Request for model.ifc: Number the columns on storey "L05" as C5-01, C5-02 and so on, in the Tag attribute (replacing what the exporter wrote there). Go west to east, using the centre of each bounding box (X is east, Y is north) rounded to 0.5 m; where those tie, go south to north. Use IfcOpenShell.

First a look at what the model holds.

```python
import ifcopenshell
import ifcopenshell.util.element
import ifcopenshell.util.placement

model = ifcopenshell.open("model.ifc")
print(model.schema)
storey = next(s for s in model.by_type("IfcBuildingStorey") if s.Name == "L05")
columns = [e for e in ifcopenshell.util.element.get_decomposition(storey) if e.is_a("IfcColumn")]
for e in sorted(columns, key=lambda e: e.id()):
    origin = ifcopenshell.util.placement.get_local_placement(e.ObjectPlacement)[:3, 3]
    print(e.id(), e.Tag, e.Name, origin.round(2) + 0.0, sep=" | ")
```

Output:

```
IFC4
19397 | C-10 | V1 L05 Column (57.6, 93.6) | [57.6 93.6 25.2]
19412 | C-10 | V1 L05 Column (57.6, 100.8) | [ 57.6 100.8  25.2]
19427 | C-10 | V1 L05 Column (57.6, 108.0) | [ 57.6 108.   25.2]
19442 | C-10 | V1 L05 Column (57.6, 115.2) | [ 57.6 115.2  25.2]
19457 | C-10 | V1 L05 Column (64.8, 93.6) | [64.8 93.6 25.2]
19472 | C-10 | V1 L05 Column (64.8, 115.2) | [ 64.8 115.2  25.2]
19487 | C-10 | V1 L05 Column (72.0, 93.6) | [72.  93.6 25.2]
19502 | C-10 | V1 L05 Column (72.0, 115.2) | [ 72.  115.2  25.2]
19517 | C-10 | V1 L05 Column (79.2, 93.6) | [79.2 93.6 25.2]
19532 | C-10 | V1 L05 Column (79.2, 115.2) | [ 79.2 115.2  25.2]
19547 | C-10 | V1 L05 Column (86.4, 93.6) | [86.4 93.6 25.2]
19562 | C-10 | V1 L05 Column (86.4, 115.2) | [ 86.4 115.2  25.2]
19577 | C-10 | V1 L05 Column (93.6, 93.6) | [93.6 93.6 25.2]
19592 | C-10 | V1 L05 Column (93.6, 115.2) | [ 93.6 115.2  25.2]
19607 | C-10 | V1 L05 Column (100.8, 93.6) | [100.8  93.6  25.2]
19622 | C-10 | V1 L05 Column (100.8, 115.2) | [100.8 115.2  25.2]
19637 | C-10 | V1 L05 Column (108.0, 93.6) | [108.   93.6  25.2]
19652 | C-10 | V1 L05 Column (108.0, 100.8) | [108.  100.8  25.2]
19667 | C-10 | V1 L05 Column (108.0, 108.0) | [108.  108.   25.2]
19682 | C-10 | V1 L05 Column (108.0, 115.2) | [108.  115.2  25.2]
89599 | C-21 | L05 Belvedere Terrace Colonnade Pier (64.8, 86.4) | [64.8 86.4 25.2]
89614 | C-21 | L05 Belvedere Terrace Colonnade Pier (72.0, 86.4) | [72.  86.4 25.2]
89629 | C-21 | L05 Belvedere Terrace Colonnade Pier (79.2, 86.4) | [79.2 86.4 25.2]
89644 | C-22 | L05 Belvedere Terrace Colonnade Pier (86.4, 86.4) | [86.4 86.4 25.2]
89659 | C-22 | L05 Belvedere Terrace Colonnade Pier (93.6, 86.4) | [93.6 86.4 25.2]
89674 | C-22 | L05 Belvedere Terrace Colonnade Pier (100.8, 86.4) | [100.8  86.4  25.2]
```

```python
import ifcopenshell
import ifcopenshell.geom
import ifcopenshell.util.element
import ifcopenshell.util.shape

model = ifcopenshell.open("model.ifc")
settings = ifcopenshell.geom.settings()
settings.set("use-world-coords", True)


def centre(element):
    shape = ifcopenshell.geom.create_shape(settings, element)
    return ifcopenshell.util.shape.get_bbox_centroid(shape.geometry)


storey = next(s for s in model.by_type("IfcBuildingStorey") if s.Name == "L05")
columns = [e for e in ifcopenshell.util.element.get_decomposition(storey) if e.is_a("IfcColumn")]

# Insertion points can sit at a corner or the storey origin, so sort by the geometry (in metres).
centres = {e: centre(e) for e in columns}
columns.sort(key=lambda e: (round(centres[e][0] / 0.5), centres[e][1]))

for i, e in enumerate(columns, start=1):
    number = f"C5-{i:02d}"
    e.Tag = number
    print(e.id(), number)

model.write("model_v2.ifc")
```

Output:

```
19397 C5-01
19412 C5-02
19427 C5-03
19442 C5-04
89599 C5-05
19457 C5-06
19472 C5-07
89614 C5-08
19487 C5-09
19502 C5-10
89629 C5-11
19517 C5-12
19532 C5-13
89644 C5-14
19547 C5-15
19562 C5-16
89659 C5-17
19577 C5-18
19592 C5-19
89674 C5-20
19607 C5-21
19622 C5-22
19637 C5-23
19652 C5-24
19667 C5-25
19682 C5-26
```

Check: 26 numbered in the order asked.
